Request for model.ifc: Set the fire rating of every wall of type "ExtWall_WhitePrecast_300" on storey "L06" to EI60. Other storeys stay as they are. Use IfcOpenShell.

First a look at what the model holds.

```python
import ifcopenshell
import ifcopenshell.util.element

model = ifcopenshell.open("model.ifc")
print(model.schema)
storey = next(s for s in model.by_type("IfcBuildingStorey") if s.Name == "L06")
walls = [e for e in ifcopenshell.util.element.get_decomposition(storey) if e.is_a("IfcWall")]
seen = {}
for e in walls:
    element_type = ifcopenshell.util.element.get_type(e)
    key = (element_type.Name if element_type != e and element_type else None, ifcopenshell.util.element.get_pset(e, "Pset_WallCommon", "FireRating"))
    seen[key] = seen.get(key, 0) + 1
for (name, value), count in sorted(seen.items(), key=str):
    print(count, "x", name, "|", value)
```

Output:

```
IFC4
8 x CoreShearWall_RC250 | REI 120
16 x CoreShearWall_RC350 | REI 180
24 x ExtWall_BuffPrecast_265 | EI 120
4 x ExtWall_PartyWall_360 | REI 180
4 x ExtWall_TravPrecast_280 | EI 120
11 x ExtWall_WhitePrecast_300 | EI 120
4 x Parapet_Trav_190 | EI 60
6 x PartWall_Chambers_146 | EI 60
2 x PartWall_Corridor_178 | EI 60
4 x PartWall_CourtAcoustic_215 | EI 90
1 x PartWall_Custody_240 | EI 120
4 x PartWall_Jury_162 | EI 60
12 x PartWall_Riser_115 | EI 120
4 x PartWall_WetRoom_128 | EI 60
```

```python
import ifcopenshell
import ifcopenshell.api.pset
import ifcopenshell.util.element

model = ifcopenshell.open("model.ifc")

storey = next(s for s in model.by_type("IfcBuildingStorey") if s.Name == "L06")
walls = [e for e in ifcopenshell.util.element.get_decomposition(storey) if e.is_a("IfcWall")]

count = 0
for e in walls:
    element_type = ifcopenshell.util.element.get_type(e)
    if element_type in (None, e) or element_type.Name != "ExtWall_WhitePrecast_300":
        continue
    # add_pset returns the element's existing set when there is one.
    pset = ifcopenshell.api.pset.add_pset(model, product=e, name="Pset_WallCommon")
    ifcopenshell.api.pset.edit_pset(model, pset=pset, properties={"FireRating": "EI60"})
    count += 1

print(count, "walls updated")

model.write("model-out.ifc")
```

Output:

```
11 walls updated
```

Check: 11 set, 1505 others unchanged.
